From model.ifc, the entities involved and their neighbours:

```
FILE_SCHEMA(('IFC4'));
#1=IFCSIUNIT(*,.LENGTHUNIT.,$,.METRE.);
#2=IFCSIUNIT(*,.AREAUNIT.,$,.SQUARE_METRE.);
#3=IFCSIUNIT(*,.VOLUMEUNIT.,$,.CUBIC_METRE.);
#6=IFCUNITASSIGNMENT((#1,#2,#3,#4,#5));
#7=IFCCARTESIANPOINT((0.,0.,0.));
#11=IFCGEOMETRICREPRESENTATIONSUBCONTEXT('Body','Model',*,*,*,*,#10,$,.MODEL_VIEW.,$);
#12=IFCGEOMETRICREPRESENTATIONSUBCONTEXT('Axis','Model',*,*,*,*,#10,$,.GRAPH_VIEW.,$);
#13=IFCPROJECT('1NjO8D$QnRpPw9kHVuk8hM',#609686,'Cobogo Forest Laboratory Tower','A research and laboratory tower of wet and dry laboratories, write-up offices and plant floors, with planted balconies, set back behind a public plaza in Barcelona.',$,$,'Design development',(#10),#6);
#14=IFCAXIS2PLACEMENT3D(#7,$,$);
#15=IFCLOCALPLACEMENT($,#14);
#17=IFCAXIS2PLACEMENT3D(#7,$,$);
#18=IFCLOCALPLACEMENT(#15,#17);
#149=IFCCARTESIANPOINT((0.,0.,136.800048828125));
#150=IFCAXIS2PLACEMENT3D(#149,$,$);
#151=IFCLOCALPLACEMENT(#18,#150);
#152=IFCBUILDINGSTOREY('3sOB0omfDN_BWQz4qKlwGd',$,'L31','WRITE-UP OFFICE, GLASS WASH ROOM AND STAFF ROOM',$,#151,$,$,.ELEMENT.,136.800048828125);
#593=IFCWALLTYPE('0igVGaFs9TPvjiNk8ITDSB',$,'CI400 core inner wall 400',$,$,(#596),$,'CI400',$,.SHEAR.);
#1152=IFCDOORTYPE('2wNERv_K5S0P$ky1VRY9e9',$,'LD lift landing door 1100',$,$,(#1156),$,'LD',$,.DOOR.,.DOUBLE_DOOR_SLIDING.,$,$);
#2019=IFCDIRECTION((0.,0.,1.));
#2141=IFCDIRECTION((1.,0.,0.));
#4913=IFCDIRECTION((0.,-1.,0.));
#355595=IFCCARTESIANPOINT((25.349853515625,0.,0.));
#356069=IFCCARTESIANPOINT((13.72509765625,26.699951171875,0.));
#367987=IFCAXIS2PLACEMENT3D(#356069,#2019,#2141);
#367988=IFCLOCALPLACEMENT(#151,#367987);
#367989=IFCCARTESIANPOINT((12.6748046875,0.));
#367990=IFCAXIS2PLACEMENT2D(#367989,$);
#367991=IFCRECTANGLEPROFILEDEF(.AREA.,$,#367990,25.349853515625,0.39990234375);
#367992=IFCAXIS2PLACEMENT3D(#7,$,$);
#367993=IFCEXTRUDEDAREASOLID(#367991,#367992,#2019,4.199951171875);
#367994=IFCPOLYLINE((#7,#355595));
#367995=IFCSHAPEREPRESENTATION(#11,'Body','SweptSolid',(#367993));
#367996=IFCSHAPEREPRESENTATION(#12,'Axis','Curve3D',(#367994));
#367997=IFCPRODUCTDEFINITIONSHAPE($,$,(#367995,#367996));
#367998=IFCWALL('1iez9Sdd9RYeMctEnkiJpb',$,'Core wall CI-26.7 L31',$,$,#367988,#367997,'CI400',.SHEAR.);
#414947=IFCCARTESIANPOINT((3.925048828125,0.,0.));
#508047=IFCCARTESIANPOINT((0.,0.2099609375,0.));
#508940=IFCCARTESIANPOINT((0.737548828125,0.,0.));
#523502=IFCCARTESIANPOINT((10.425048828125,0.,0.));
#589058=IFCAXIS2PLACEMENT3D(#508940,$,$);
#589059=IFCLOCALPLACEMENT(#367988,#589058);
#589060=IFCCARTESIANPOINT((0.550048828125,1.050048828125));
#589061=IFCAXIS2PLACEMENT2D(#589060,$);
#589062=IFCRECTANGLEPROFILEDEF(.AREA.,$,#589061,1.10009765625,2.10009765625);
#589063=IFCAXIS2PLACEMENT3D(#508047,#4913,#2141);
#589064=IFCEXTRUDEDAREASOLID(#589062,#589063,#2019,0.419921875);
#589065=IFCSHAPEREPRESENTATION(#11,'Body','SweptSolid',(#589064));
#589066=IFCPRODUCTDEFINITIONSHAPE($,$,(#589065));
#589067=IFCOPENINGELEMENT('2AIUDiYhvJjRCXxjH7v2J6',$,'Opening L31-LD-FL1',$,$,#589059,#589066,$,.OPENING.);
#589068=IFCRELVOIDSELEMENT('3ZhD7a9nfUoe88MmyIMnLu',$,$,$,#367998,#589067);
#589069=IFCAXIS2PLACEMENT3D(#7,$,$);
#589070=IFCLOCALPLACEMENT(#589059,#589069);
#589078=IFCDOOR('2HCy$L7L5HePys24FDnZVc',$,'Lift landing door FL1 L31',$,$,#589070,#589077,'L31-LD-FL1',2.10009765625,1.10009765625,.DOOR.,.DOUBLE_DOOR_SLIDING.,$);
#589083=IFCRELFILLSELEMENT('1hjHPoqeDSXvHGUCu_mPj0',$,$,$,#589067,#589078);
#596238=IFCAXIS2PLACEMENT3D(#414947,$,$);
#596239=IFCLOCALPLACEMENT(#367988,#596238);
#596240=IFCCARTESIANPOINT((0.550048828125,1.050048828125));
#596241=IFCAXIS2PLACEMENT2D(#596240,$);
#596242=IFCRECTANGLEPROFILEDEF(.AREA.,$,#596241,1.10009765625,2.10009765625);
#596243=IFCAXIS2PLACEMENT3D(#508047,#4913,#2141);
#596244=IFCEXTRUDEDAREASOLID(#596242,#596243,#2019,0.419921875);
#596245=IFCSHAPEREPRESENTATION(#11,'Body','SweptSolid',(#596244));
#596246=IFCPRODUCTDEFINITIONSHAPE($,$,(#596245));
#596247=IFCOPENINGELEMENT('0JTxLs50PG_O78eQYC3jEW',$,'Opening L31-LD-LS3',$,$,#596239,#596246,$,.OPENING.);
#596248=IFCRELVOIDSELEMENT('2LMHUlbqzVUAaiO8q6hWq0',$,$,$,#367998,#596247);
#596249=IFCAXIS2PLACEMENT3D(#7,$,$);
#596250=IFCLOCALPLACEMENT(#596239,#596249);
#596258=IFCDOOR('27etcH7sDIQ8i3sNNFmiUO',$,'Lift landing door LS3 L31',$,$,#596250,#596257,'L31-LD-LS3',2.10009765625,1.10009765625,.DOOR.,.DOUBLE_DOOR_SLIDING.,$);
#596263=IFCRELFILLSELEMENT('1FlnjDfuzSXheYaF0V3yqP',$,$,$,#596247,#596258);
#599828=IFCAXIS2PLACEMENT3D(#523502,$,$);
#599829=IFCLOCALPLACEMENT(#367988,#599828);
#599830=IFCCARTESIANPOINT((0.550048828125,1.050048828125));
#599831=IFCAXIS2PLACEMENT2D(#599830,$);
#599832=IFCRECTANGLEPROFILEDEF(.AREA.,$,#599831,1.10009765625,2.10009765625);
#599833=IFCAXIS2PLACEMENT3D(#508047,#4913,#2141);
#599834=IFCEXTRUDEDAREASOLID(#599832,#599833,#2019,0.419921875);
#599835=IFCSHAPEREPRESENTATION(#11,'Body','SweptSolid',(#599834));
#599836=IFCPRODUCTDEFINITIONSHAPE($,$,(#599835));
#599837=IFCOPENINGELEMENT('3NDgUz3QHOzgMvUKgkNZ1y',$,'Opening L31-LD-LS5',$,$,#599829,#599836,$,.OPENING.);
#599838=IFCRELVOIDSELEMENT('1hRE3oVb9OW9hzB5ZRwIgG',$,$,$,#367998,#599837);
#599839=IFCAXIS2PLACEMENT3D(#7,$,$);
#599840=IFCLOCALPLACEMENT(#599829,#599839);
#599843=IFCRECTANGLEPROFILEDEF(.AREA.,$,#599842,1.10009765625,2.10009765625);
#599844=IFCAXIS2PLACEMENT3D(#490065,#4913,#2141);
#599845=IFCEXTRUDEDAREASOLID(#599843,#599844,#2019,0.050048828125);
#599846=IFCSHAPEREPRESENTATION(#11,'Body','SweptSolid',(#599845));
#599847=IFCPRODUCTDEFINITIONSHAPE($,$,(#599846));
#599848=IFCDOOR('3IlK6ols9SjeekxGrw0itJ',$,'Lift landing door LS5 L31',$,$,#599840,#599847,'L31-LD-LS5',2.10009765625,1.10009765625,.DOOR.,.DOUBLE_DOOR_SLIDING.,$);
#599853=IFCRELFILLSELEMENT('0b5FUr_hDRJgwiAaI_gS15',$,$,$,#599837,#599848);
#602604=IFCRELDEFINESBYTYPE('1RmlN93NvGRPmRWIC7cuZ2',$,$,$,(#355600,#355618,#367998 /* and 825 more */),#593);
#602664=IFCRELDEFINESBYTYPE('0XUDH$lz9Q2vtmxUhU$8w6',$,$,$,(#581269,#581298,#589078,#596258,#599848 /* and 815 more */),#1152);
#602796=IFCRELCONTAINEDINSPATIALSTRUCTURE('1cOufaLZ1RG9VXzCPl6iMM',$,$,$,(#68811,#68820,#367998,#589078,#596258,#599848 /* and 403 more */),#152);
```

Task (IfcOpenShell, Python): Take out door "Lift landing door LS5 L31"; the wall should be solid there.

```python
import ifcopenshell
import ifcopenshell.api.feature
import ifcopenshell.api.root
import ifcopenshell.geom
import ifcopenshell.util.shape

model = ifcopenshell.open("model.ifc")
settings = ifcopenshell.geom.settings()


def volume(element):
    """Net volume in cubic metres, openings subtracted."""
    shape = ifcopenshell.geom.create_shape(settings, element)
    return ifcopenshell.util.shape.get_volume(shape.geometry)


door = model.by_guid("3IlK6ols9SjeekxGrw0itJ")
opening = door.FillsVoids[0].RelatingOpeningElement
wall = opening.VoidsElements[0].RelatingBuildingElement
before = volume(wall)

ifcopenshell.api.root.remove_product(model, product=door)
ifcopenshell.api.feature.remove_feature(model, feature=opening)

after = volume(wall)

print(f"wall volume {before:.3f} -> {after:.3f} m3")

model.write("model_rev.ifc")
```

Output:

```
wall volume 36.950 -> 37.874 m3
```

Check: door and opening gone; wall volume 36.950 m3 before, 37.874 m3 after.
